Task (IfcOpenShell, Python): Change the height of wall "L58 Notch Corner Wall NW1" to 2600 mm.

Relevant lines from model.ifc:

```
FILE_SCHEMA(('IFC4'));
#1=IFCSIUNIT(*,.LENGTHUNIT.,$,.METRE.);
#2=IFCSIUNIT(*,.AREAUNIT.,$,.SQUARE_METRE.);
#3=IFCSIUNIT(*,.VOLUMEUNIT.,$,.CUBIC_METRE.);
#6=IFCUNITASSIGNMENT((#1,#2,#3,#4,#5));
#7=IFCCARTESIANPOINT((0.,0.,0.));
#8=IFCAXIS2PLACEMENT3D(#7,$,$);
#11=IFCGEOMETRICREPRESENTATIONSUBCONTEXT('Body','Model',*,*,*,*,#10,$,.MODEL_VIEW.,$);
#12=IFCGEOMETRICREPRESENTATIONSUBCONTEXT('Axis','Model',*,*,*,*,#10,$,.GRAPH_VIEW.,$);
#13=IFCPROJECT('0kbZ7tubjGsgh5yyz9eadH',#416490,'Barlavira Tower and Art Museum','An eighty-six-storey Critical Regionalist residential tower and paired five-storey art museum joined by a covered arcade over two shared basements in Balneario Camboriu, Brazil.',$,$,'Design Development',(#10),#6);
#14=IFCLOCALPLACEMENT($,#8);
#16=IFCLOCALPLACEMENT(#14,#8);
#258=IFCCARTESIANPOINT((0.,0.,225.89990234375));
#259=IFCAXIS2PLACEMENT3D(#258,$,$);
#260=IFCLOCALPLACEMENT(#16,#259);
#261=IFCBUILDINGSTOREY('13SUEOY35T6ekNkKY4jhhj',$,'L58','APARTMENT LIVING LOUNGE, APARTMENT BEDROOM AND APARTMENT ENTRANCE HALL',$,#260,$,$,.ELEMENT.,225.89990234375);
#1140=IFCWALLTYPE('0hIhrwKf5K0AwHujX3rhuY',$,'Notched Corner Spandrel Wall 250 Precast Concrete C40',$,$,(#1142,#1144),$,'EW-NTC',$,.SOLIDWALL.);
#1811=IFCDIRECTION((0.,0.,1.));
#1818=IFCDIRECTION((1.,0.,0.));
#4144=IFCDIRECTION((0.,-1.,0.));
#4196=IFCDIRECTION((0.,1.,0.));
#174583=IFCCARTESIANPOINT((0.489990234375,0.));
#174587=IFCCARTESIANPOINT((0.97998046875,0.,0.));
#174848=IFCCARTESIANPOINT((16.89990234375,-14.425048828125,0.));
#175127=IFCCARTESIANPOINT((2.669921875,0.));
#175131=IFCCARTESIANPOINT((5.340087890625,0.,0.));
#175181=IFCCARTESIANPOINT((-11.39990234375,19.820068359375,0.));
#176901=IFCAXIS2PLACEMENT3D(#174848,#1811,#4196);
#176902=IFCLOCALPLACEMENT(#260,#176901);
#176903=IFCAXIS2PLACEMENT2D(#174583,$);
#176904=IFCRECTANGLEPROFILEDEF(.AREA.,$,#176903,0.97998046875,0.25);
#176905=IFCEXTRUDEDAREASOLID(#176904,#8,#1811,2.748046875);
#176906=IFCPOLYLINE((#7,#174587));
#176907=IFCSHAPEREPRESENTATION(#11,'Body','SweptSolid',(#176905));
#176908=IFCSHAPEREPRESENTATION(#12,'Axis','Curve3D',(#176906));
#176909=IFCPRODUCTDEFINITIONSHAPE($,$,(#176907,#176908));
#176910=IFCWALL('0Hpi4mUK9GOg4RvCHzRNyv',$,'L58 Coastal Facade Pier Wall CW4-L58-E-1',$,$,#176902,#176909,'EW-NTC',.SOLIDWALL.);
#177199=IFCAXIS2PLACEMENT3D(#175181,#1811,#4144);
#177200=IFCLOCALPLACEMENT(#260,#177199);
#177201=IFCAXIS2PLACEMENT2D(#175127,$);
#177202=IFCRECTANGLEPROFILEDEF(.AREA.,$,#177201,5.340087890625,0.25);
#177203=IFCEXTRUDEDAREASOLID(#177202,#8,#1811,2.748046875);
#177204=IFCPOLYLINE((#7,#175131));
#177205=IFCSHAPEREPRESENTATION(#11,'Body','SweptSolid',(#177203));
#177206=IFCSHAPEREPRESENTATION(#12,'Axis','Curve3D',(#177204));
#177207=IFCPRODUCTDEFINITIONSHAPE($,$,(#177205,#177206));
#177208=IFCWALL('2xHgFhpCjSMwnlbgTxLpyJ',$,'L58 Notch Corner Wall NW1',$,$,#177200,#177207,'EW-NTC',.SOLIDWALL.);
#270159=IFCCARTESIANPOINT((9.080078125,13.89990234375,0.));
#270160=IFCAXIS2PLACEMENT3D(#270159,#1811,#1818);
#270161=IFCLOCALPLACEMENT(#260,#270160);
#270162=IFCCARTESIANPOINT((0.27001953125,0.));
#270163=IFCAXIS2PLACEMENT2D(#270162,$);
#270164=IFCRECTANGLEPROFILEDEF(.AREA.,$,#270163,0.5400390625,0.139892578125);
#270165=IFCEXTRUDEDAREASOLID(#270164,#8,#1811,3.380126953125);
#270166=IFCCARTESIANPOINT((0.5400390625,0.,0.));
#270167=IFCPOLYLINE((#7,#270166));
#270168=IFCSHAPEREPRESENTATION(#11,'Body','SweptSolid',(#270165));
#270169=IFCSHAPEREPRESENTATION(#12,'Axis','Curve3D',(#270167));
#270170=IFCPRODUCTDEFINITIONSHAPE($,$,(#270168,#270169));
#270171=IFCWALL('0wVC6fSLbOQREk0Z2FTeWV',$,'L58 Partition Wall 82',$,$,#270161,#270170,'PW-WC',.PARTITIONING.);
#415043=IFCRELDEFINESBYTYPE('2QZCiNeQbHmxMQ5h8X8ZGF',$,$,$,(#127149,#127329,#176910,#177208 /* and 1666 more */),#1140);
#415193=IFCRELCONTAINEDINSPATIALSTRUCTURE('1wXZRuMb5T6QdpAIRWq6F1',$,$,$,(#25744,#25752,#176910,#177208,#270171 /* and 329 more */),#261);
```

```python
import ifcopenshell
import ifcopenshell.geom
import ifcopenshell.util.representation
import ifcopenshell.util.shape

model = ifcopenshell.open("model.ifc")
settings = ifcopenshell.geom.settings()


def volume(element):
    """Net volume in cubic metres, openings subtracted."""
    shape = ifcopenshell.geom.create_shape(settings, element)
    return ifcopenshell.util.shape.get_volume(shape.geometry)


wall = model.by_guid("2xHgFhpCjSMwnlbgTxLpyJ")
before = volume(wall)

body = ifcopenshell.util.representation.get_representation(wall, "Model", "Body")
solid = body.Items[0]
old_height = solid.Depth
solid.Depth = 2.6
after = volume(wall)

print(f"height {old_height:g} -> {solid.Depth:g}, volume {before:.3f} -> {after:.3f} m3")

model.write("model_updated.ifc")
```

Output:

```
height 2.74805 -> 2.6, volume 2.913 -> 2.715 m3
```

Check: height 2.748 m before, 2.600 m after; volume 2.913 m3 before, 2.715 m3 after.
